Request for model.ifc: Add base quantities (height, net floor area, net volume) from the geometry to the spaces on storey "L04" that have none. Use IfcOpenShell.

First a look at what the model holds.

```python
import ifcopenshell
import ifcopenshell.util.element
import ifcopenshell.util.unit

model = ifcopenshell.open("model.ifc")
print(model.schema)
for unit_type in ("LENGTHUNIT", "AREAUNIT", "VOLUMEUNIT"):
    print(unit_type, ifcopenshell.util.unit.calculate_unit_scale(model, unit_type))
storey = next(s for s in model.by_type("IfcBuildingStorey") if s.Name == "L04")
spaces = [e for e in ifcopenshell.util.element.get_decomposition(storey) if e.is_a("IfcSpace")]
for e in sorted(spaces, key=lambda e: e.id()):
    print(e.id(), e.is_a(), e.Name, list(ifcopenshell.util.element.get_psets(e, qtos_only=True)), sep=" | ")
```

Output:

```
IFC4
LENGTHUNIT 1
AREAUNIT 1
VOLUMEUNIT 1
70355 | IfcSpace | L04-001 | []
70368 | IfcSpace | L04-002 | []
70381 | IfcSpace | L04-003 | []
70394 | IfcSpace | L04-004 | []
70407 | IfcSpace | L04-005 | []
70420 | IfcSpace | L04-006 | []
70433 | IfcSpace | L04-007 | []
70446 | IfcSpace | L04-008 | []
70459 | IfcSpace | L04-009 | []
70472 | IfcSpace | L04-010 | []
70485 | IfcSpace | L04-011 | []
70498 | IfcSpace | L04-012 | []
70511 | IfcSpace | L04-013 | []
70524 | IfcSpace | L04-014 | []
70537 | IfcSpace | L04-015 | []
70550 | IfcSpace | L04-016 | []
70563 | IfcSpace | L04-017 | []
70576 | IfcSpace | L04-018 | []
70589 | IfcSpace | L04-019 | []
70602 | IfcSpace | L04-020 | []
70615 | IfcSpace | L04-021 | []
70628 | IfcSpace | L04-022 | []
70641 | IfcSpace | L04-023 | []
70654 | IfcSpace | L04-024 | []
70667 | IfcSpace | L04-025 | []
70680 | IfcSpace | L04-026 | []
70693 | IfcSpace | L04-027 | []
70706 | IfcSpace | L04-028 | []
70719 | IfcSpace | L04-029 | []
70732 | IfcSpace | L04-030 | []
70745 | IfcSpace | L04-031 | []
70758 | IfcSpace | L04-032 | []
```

```python
import ifcopenshell
import ifcopenshell.api.pset
import ifcopenshell.geom
import ifcopenshell.util.element
import ifcopenshell.util.shape
import ifcopenshell.util.unit

model = ifcopenshell.open("model.ifc")
unit_scale = ifcopenshell.util.unit.calculate_unit_scale(model)
area_scale = ifcopenshell.util.unit.calculate_unit_scale(model, "AREAUNIT")
volume_scale = ifcopenshell.util.unit.calculate_unit_scale(model, "VOLUMEUNIT")
settings = ifcopenshell.geom.settings()

storey = next(s for s in model.by_type("IfcBuildingStorey") if s.Name == "L04")
spaces = [e for e in ifcopenshell.util.element.get_decomposition(storey) if e.is_a("IfcSpace")]

for e in sorted(spaces, key=lambda e: e.id()):
    if ifcopenshell.util.element.get_psets(e, qtos_only=True, should_inherit=False):
        continue
    # Geometry comes back in metres, in the element's own axes.
    shape = ifcopenshell.geom.create_shape(settings, e)
    values = {
        "Height": ifcopenshell.util.shape.get_z(shape.geometry) / unit_scale,
        "NetFloorArea": ifcopenshell.util.shape.get_footprint_area(shape.geometry) / area_scale,
        "NetVolume": ifcopenshell.util.shape.get_volume(shape.geometry) / volume_scale,
    }
    qto = ifcopenshell.api.pset.add_qto(model, product=e, name="Qto_SpaceBaseQuantities")
    ifcopenshell.api.pset.edit_qto(model, qto=qto, properties=values)
    print(e.id(), {k: round(v, 3) for k, v in values.items()})

model.write("model_v2.ifc")
```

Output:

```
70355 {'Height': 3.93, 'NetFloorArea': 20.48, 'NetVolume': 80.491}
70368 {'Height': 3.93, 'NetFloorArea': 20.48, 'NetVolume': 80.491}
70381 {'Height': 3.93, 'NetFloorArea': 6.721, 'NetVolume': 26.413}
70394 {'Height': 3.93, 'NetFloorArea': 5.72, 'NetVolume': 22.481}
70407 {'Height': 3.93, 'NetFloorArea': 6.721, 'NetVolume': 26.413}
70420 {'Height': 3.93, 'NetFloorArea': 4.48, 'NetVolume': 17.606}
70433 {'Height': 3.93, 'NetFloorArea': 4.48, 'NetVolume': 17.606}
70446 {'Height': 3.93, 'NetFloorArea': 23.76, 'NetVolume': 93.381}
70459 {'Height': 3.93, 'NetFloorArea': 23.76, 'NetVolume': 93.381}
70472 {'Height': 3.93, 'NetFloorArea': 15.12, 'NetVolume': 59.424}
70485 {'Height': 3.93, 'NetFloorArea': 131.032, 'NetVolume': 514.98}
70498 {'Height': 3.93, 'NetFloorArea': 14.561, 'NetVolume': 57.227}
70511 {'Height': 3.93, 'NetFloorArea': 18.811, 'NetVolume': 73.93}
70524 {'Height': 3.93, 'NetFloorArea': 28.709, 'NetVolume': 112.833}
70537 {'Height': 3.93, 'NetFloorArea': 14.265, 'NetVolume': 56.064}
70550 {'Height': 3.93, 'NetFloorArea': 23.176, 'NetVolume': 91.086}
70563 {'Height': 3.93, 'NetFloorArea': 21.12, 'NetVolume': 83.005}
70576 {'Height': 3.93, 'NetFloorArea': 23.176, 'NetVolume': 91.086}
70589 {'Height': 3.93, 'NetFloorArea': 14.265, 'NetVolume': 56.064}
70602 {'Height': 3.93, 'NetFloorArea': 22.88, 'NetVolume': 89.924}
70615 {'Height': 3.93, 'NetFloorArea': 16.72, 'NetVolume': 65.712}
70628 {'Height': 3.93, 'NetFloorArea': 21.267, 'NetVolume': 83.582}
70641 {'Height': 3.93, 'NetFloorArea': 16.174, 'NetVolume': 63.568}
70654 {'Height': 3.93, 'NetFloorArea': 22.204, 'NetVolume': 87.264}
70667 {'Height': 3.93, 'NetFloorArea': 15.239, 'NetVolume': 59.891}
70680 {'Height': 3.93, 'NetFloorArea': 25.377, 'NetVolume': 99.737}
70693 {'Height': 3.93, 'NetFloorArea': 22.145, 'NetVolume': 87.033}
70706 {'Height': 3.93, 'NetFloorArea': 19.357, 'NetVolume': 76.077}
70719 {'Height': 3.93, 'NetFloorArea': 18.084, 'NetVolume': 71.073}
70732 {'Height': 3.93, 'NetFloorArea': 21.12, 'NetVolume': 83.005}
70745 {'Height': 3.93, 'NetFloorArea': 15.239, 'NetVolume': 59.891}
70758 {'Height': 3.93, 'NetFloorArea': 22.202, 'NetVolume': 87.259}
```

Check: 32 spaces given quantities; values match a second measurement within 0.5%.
